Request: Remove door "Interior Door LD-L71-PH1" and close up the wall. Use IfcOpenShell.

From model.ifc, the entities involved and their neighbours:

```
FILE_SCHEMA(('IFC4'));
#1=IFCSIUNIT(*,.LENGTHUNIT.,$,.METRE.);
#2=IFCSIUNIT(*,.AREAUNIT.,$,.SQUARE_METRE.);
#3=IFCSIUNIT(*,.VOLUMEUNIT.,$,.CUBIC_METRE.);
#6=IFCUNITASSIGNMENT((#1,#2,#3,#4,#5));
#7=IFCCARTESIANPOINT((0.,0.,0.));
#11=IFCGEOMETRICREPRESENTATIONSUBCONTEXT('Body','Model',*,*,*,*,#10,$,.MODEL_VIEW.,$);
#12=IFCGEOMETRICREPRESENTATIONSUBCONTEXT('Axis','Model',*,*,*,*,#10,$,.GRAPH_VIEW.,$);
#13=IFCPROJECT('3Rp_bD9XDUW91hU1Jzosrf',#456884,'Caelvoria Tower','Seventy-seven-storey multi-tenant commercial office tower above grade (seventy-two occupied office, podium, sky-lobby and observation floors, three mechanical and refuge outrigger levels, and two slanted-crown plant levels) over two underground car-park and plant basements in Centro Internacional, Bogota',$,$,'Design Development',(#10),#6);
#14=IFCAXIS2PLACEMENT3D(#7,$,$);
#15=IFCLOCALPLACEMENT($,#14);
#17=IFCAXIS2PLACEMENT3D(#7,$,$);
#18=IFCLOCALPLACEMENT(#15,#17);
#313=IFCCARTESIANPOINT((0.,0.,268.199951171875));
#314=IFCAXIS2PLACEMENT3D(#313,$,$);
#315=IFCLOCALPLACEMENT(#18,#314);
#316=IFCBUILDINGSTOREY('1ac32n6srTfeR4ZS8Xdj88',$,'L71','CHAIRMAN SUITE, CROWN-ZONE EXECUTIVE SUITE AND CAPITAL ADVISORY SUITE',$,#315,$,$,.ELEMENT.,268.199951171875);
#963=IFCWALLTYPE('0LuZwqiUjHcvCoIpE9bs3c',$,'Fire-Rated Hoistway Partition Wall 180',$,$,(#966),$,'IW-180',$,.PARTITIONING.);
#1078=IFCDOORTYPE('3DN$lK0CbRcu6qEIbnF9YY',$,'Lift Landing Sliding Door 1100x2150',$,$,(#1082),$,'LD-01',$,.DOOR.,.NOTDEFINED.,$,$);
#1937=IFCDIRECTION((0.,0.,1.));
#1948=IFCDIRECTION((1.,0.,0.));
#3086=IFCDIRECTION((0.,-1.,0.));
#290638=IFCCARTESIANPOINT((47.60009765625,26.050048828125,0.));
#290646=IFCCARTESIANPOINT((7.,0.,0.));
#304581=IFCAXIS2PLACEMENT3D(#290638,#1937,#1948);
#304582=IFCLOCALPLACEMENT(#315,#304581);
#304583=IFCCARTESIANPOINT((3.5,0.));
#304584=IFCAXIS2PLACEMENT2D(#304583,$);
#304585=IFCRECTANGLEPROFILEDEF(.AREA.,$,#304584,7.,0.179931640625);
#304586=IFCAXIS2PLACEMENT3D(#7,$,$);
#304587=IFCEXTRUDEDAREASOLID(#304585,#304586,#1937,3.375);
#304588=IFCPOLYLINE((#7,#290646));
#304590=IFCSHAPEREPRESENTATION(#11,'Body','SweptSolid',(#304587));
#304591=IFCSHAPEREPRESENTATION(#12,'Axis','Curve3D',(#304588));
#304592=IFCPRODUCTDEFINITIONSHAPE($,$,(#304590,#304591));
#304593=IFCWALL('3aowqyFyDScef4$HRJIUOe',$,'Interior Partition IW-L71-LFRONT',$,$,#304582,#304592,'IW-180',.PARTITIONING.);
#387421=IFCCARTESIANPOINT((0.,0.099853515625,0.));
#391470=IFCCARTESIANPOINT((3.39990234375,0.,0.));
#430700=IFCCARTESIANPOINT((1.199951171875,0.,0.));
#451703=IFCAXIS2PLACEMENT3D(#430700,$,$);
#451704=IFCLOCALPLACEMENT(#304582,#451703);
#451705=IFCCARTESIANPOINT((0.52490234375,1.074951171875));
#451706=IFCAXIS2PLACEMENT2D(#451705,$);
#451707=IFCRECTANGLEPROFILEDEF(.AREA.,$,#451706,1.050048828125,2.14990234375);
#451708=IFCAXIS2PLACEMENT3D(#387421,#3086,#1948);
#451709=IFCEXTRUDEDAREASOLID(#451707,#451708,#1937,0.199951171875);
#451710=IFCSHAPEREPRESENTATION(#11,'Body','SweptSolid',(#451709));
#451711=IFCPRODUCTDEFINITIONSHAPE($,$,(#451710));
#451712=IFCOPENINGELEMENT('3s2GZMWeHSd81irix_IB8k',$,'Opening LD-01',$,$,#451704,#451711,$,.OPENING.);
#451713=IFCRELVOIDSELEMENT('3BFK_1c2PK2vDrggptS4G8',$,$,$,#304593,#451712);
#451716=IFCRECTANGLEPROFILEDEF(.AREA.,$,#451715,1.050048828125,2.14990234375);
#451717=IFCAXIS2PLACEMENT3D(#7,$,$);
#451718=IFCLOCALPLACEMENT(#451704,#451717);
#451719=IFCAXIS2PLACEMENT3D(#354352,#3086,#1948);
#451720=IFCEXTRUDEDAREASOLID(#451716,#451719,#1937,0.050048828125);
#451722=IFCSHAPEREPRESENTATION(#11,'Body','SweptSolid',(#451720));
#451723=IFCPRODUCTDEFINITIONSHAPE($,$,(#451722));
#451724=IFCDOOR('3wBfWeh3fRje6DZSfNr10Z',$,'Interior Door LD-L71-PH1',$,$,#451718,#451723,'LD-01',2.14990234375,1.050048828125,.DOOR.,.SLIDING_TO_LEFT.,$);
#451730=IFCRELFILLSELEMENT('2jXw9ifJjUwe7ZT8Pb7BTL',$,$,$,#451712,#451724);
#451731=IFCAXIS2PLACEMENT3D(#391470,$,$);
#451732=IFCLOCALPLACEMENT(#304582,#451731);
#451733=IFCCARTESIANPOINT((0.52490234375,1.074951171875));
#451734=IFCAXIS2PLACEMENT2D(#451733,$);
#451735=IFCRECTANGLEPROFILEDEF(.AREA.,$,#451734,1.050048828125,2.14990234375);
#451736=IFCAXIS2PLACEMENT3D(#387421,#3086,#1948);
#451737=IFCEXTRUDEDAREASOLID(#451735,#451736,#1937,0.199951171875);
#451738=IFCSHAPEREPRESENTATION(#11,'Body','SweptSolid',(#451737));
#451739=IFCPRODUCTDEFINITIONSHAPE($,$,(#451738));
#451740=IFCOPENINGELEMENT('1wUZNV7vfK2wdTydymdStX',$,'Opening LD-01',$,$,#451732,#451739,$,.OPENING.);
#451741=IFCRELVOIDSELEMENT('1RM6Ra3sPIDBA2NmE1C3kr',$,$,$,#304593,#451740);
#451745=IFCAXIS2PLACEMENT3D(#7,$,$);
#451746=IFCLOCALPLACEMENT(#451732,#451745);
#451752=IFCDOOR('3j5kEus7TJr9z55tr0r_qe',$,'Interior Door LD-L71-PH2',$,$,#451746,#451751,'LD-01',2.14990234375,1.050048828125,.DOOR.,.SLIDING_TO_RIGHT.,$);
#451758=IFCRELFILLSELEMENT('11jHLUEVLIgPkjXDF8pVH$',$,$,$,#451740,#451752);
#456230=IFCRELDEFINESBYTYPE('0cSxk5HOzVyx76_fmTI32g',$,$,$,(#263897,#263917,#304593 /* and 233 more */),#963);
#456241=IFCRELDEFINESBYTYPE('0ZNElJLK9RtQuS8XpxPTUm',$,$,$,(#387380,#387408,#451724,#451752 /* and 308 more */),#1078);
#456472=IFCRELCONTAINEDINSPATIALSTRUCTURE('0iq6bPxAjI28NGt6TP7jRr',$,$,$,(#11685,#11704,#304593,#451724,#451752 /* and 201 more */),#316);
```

```python
import ifcopenshell
import ifcopenshell.api.feature
import ifcopenshell.api.root
import ifcopenshell.geom
import ifcopenshell.util.shape

model = ifcopenshell.open("model.ifc")
settings = ifcopenshell.geom.settings()


def volume(element):
    """Net volume in cubic metres, openings subtracted."""
    shape = ifcopenshell.geom.create_shape(settings, element)
    return ifcopenshell.util.shape.get_volume(shape.geometry)


door = model.by_id(451724)
opening = door.FillsVoids[0].RelatingOpeningElement
wall = opening.VoidsElements[0].RelatingBuildingElement
before = volume(wall)

ifcopenshell.api.root.remove_product(model, product=door)
ifcopenshell.api.feature.remove_feature(model, feature=opening)

after = volume(wall)

print(f"wall volume {before:.3f} -> {after:.3f} m3")

model.write("model_edited.ifc")
```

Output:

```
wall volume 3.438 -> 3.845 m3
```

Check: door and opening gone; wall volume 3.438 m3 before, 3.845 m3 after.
